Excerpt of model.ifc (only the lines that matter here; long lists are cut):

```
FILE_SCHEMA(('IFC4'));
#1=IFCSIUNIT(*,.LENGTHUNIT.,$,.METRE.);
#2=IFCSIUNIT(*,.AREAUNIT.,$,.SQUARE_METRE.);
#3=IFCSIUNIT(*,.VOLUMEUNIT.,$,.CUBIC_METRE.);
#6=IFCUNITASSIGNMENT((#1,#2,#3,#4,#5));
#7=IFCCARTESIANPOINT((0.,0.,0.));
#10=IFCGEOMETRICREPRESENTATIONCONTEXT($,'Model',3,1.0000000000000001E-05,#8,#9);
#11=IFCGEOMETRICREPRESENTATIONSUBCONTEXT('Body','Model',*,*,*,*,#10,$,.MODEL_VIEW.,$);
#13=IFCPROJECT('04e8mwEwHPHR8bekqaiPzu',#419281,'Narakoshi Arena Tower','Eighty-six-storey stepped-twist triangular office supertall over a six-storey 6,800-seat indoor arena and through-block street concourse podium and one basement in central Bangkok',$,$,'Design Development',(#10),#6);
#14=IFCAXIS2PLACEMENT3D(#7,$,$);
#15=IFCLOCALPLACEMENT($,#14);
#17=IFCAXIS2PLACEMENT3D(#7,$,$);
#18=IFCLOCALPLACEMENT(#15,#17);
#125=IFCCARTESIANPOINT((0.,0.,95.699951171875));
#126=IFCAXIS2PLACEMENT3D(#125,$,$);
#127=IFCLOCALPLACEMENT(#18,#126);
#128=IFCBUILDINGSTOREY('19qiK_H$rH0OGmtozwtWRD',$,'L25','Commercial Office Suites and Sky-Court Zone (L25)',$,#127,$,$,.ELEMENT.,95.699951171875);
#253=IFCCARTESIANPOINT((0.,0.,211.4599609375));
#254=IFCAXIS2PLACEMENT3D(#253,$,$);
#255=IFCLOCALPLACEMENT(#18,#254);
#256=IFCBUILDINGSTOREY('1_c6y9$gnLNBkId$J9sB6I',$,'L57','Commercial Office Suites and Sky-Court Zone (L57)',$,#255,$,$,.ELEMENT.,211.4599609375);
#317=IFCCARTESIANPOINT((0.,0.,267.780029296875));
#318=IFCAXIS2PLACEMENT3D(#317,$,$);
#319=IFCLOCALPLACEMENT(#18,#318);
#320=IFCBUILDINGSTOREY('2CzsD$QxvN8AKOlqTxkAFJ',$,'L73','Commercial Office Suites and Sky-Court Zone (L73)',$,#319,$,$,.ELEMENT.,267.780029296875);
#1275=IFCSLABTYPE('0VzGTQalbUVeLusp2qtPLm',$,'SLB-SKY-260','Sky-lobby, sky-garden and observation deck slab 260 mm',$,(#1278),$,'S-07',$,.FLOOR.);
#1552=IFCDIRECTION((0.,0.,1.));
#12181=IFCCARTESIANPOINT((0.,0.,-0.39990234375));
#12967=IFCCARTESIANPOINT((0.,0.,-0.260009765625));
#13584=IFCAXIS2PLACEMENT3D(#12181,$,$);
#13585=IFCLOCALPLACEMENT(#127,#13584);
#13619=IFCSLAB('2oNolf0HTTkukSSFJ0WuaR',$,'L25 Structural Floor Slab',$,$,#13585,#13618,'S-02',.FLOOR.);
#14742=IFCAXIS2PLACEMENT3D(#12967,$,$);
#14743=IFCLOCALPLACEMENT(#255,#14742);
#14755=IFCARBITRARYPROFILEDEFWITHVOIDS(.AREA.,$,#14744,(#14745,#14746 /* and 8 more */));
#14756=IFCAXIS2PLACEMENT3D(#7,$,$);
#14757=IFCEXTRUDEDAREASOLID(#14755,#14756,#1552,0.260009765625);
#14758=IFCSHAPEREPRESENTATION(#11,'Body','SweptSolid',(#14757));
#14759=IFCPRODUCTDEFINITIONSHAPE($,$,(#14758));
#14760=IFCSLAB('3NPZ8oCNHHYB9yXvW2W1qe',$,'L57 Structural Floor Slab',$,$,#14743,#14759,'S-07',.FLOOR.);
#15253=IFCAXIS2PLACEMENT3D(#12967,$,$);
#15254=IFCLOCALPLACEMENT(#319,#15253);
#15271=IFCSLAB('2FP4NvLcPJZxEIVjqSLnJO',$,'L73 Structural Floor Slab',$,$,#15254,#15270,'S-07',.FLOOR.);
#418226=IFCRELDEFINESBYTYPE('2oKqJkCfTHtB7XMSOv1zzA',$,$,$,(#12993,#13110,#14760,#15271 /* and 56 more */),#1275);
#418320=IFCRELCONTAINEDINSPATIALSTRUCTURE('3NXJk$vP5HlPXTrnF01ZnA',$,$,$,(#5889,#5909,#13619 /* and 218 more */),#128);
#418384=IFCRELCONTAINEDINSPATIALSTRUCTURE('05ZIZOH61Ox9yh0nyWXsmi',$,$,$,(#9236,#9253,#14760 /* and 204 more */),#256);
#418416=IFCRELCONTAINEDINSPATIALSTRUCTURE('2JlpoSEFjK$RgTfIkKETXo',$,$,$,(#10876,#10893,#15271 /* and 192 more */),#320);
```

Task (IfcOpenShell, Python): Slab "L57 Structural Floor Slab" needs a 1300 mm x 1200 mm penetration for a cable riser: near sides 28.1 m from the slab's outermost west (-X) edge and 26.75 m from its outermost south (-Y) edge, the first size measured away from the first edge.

```python
import numpy as np
import ifcopenshell
import ifcopenshell.api.feature
import ifcopenshell.api.geometry
import ifcopenshell.api.root
import ifcopenshell.geom
import ifcopenshell.util.placement
import ifcopenshell.util.representation
import ifcopenshell.util.shape
import ifcopenshell.util.unit

model = ifcopenshell.open("model.ifc")
unit_scale = ifcopenshell.util.unit.calculate_unit_scale(model)
settings = ifcopenshell.geom.settings()


def volume(element):
    """Net volume in cubic metres, openings subtracted."""
    shape = ifcopenshell.geom.create_shape(settings, element)
    return ifcopenshell.util.shape.get_volume(shape.geometry)


slab = model.by_guid("3NPZ8oCNHHYB9yXvW2W1qe")
before = volume(slab)

# Extent in the slab's own axes, in metres. The edges named are its -X and -Y sides.
slab_shape = ifcopenshell.geom.create_shape(settings, slab)
vertices = ifcopenshell.util.shape.get_vertices(slab_shape.geometry)
x_min, y_min, bottom = vertices.min(axis=0)
top = vertices[:, 2].max()

opening = ifcopenshell.api.root.create_entity(model, ifc_class="IfcOpeningElement", name="Cable riser opening", predefined_type="OPENING")
context = ifcopenshell.util.representation.get_context(model, "Model", "Body", "MODEL_VIEW")
width, depth = 1.3, 1.2
outline = [(0.0, 0.0), (width, 0.0), (width, depth), (0.0, depth), (0.0, 0.0)]
# Overshoot both faces by 50 mm so the cut is clean.
shape = ifcopenshell.api.geometry.add_slab_representation(
    model, context=context, depth=top - bottom + 0.1, polyline=outline
)
ifcopenshell.api.geometry.assign_representation(model, product=opening, representation=shape)

matrix = ifcopenshell.util.placement.get_local_placement(slab.ObjectPlacement)
matrix[:, 3] = matrix @ np.append(np.array([x_min + 28.1, y_min + 26.75, bottom - 0.05]) / unit_scale, 1.0)
ifcopenshell.api.geometry.edit_object_placement(model, product=opening, matrix=matrix, is_si=False)
ifcopenshell.api.feature.add_feature(model, feature=opening, element=slab)

after = volume(slab)

print(f"slab volume {before:.3f} -> {after:.3f} m3")

model.write("model_edited.ifc")
```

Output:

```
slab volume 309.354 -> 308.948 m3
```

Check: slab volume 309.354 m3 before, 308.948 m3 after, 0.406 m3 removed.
